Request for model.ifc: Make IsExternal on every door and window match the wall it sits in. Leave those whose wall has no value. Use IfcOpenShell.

First a look at what the model holds.

```python
import ifcopenshell
import ifcopenshell.util.element

model = ifcopenshell.open("model.ifc")
print(model.schema)
seen = {}
for e in model.by_type("IfcDoor") + model.by_type("IfcWindow"):
    if not e.FillsVoids:
        continue
    host = e.FillsVoids[0].RelatingOpeningElement.VoidsElements[0].RelatingBuildingElement
    own = ifcopenshell.util.element.get_pset(e, f"Pset_{e.is_a()[3:].removesuffix('StandardCase')}Common", "IsExternal")
    wall = ifcopenshell.util.element.get_pset(host, "Pset_WallCommon", "IsExternal")
    seen[e.is_a(), own, wall] = seen.get((e.is_a(), own, wall), 0) + 1
for (cls, own, wall), count in sorted(seen.items(), key=str):
    print(count, cls, "IsExternal:", own, "| host wall:", wall)
```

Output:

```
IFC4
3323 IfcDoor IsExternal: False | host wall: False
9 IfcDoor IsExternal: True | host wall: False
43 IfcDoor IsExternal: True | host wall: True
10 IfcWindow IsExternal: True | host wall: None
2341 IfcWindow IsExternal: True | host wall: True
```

```python
import ifcopenshell
import ifcopenshell.api.pset
import ifcopenshell.util.element

model = ifcopenshell.open("model.ifc")

count = 0
for ifc_class, pset_name in (("IfcDoor", "Pset_DoorCommon"), ("IfcWindow", "Pset_WindowCommon")):
    for e in model.by_type(ifc_class):
        if not e.FillsVoids:
            continue
        host = e.FillsVoids[0].RelatingOpeningElement.VoidsElements[0].RelatingBuildingElement
        external = ifcopenshell.util.element.get_pset(host, "Pset_WallCommon", "IsExternal")
        if external is None or ifcopenshell.util.element.get_pset(e, pset_name, "IsExternal") == external:
            continue
        pset = ifcopenshell.api.pset.add_pset(model, product=e, name=pset_name)
        ifcopenshell.api.pset.edit_pset(model, pset=pset, properties={"IsExternal": external})
        count += 1

print(count, "updated")

model.write("model_edited.ifc")
```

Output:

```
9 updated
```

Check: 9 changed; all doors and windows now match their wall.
